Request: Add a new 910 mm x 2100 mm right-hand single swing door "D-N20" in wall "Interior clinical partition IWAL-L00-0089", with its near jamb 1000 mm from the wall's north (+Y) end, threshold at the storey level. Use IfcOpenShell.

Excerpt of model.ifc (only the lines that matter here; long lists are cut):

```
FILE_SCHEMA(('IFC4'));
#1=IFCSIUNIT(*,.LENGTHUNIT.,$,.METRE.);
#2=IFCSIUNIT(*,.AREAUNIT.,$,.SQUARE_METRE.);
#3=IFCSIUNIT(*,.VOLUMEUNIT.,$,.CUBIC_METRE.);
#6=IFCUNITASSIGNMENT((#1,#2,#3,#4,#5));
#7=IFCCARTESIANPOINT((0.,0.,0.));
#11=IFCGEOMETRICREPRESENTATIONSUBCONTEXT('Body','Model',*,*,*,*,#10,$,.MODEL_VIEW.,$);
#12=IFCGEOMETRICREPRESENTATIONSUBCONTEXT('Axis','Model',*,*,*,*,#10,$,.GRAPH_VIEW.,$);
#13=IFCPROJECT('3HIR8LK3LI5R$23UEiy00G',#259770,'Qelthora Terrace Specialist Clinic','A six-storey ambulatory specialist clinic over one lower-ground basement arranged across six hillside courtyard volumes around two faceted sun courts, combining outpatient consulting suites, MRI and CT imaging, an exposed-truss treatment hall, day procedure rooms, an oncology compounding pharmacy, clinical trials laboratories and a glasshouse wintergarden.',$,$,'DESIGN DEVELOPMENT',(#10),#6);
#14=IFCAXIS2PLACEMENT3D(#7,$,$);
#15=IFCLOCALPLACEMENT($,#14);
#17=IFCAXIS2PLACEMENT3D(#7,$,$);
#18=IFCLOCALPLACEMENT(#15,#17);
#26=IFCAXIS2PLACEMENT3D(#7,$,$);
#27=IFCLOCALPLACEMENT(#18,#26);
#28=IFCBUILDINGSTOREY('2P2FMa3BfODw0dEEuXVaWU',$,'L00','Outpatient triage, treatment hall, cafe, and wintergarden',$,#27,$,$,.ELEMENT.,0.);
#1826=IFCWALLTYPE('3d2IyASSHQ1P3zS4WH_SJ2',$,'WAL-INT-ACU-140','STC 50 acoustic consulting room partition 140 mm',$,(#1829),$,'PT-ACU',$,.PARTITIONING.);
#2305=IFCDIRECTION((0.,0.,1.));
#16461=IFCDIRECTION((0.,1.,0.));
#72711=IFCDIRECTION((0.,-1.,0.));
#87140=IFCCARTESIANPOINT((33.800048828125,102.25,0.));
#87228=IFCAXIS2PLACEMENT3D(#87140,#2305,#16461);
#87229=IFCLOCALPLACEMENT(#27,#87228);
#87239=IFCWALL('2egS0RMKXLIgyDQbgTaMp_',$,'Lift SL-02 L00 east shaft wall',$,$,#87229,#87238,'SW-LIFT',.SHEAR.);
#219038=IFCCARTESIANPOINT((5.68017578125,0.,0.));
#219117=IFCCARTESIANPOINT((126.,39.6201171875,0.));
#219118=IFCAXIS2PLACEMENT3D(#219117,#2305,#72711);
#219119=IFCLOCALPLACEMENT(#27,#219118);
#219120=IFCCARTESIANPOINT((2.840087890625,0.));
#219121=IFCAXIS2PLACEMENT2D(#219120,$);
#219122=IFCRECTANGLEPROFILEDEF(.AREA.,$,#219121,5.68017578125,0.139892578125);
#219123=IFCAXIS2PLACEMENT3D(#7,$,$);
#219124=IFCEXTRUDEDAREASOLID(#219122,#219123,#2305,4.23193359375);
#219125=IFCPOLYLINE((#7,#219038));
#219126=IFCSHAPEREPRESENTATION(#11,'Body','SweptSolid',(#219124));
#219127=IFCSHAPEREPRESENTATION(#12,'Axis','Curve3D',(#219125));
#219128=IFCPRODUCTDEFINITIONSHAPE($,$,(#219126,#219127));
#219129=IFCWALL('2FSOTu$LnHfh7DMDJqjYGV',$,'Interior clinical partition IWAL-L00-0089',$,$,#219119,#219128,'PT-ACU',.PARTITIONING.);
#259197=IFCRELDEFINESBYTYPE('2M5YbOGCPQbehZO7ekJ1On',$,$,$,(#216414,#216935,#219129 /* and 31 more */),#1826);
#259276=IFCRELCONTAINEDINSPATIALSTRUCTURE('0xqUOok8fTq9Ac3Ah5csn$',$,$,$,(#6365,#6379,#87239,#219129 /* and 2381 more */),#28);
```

```python
import numpy as np
import ifcopenshell
import ifcopenshell.api.feature
import ifcopenshell.api.geometry
import ifcopenshell.api.root
import ifcopenshell.api.spatial
import ifcopenshell.geom
import ifcopenshell.util.element
import ifcopenshell.util.placement
import ifcopenshell.util.representation
import ifcopenshell.util.shape
import ifcopenshell.util.unit

model = ifcopenshell.open("model.ifc")
unit_scale = ifcopenshell.util.unit.calculate_unit_scale(model)
settings = ifcopenshell.geom.settings()


def volume(element):
    """Net volume in cubic metres, openings subtracted."""
    shape = ifcopenshell.geom.create_shape(settings, element)
    return ifcopenshell.util.shape.get_volume(shape.geometry)


wall = model.by_id(219129)
storey = ifcopenshell.util.element.get_container(wall, ifc_class="IfcBuildingStorey")
context = ifcopenshell.util.representation.get_context(model, "Model", "Body", "MODEL_VIEW")
before = volume(wall)

width, height, from_end, sill = 0.91, 2.1, 1, 0.0  # metres

# The wall runs along its own X axis, and the end named is its -X end.
wall_shape = ifcopenshell.geom.create_shape(settings, wall)
x, y, z = ifcopenshell.util.shape.get_vertices(wall_shape.geometry).T
start = x.min() + from_end
face, thickness = float(y.min()), float(y.max() - y.min())
wall_matrix = ifcopenshell.util.placement.get_local_placement(wall.ObjectPlacement)
level = ifcopenshell.util.placement.get_local_placement(storey.ObjectPlacement)[2, 3]


def in_wall(x, y):
    """Placement at x, y metres in the wall's axes, at sill height."""
    matrix = wall_matrix.copy()
    matrix[:, 3] = wall_matrix @ np.array([x / unit_scale, y / unit_scale, 0.0, 1.0])
    matrix[2, 3] = level + sill / unit_scale
    return matrix


# Opening: a box that overshoots both wall faces by 50 mm.
opening = ifcopenshell.api.root.create_entity(model, ifc_class="IfcOpeningElement", predefined_type="OPENING")
box = ifcopenshell.api.geometry.add_wall_representation(
    model, context=context, length=width, height=height, thickness=thickness + 0.1
)
ifcopenshell.api.geometry.assign_representation(model, product=opening, representation=box)
ifcopenshell.api.geometry.edit_object_placement(model, product=opening, matrix=in_wall(start, face - 0.05), is_si=False)
ifcopenshell.api.feature.add_feature(model, feature=opening, element=wall)

door = ifcopenshell.api.root.create_entity(model, ifc_class="IfcDoor", name="D-N20", predefined_type="DOOR")
door.OverallWidth, door.OverallHeight = width / unit_scale, height / unit_scale
door.OperationType = "SINGLE_SWING_RIGHT"
body = ifcopenshell.api.geometry.add_door_representation(
    model,
    context=context,
    overall_width=door.OverallWidth,
    overall_height=door.OverallHeight,
    operation_type="SINGLE_SWING_RIGHT",
    lining_properties={"LiningDepth": thickness / unit_scale, "ThresholdDepth": thickness / unit_scale},
)
ifcopenshell.api.geometry.assign_representation(model, product=door, representation=body)
ifcopenshell.api.spatial.assign_container(model, products=[door], relating_structure=storey)
ifcopenshell.api.feature.add_filling(model, opening=opening, element=door)

# The lining spans the wall, so the door starts at the wall face.
ifcopenshell.api.geometry.edit_object_placement(model, product=door, matrix=in_wall(start, face), is_si=False)

after = volume(wall)

print(f"wall volume {before:.3f} -> {after:.3f} m3")

model.write("model_rev.ifc")
```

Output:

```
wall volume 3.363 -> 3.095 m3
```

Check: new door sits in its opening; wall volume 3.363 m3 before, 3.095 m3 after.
